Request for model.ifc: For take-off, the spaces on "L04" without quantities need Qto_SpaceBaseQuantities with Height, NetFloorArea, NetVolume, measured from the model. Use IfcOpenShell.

First a look at what the model holds.

```python
import ifcopenshell
import ifcopenshell.util.element
import ifcopenshell.util.unit

model = ifcopenshell.open("model.ifc")
print(model.schema)
for unit_type in ("LENGTHUNIT", "AREAUNIT", "VOLUMEUNIT"):
    print(unit_type, ifcopenshell.util.unit.calculate_unit_scale(model, unit_type))
storey = next(s for s in model.by_type("IfcBuildingStorey") if s.Name == "L04")
spaces = [e for e in ifcopenshell.util.element.get_decomposition(storey) if e.is_a("IfcSpace")]
for e in sorted(spaces, key=lambda e: e.id()):
    print(e.id(), e.is_a(), e.Name, list(ifcopenshell.util.element.get_psets(e, qtos_only=True)), sep=" | ")
```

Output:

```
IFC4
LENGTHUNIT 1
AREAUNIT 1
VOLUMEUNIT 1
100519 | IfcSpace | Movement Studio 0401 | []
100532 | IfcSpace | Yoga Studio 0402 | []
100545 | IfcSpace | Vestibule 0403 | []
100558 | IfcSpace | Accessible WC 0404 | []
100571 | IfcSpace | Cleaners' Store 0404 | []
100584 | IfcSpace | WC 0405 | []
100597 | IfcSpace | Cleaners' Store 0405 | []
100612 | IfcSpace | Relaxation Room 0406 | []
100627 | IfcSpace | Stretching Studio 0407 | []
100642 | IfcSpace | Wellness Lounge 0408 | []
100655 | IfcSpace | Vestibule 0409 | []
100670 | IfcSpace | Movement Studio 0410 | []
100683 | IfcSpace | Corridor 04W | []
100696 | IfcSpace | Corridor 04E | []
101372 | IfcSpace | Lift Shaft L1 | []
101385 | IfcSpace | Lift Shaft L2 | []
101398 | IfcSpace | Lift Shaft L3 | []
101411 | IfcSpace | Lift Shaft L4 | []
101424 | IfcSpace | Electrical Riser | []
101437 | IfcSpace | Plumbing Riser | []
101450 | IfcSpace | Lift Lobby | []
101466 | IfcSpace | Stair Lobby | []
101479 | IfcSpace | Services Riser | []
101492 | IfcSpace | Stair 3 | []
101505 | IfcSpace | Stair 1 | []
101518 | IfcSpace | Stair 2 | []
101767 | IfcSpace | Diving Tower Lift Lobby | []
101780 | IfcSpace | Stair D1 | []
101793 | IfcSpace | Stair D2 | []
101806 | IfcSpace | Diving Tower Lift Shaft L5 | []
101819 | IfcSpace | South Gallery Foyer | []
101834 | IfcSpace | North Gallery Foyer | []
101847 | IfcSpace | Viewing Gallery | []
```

```python
import ifcopenshell
import ifcopenshell.api.pset
import ifcopenshell.geom
import ifcopenshell.util.element
import ifcopenshell.util.shape
import ifcopenshell.util.unit

model = ifcopenshell.open("model.ifc")
unit_scale = ifcopenshell.util.unit.calculate_unit_scale(model)
area_scale = ifcopenshell.util.unit.calculate_unit_scale(model, "AREAUNIT")
volume_scale = ifcopenshell.util.unit.calculate_unit_scale(model, "VOLUMEUNIT")
settings = ifcopenshell.geom.settings()

storey = next(s for s in model.by_type("IfcBuildingStorey") if s.Name == "L04")
spaces = [e for e in ifcopenshell.util.element.get_decomposition(storey) if e.is_a("IfcSpace")]

for e in sorted(spaces, key=lambda e: e.id()):
    if ifcopenshell.util.element.get_psets(e, qtos_only=True, should_inherit=False):
        continue
    # Geometry comes back in metres, in the element's own axes.
    shape = ifcopenshell.geom.create_shape(settings, e)
    values = {
        "Height": ifcopenshell.util.shape.get_z(shape.geometry) / unit_scale,
        "NetFloorArea": ifcopenshell.util.shape.get_footprint_area(shape.geometry) / area_scale,
        "NetVolume": ifcopenshell.util.shape.get_volume(shape.geometry) / volume_scale,
    }
    qto = ifcopenshell.api.pset.add_qto(model, product=e, name="Qto_SpaceBaseQuantities")
    ifcopenshell.api.pset.edit_qto(model, qto=qto, properties=values)
    print(e.id(), {k: round(v, 3) for k, v in values.items()})

model.write("model-out.ifc")
```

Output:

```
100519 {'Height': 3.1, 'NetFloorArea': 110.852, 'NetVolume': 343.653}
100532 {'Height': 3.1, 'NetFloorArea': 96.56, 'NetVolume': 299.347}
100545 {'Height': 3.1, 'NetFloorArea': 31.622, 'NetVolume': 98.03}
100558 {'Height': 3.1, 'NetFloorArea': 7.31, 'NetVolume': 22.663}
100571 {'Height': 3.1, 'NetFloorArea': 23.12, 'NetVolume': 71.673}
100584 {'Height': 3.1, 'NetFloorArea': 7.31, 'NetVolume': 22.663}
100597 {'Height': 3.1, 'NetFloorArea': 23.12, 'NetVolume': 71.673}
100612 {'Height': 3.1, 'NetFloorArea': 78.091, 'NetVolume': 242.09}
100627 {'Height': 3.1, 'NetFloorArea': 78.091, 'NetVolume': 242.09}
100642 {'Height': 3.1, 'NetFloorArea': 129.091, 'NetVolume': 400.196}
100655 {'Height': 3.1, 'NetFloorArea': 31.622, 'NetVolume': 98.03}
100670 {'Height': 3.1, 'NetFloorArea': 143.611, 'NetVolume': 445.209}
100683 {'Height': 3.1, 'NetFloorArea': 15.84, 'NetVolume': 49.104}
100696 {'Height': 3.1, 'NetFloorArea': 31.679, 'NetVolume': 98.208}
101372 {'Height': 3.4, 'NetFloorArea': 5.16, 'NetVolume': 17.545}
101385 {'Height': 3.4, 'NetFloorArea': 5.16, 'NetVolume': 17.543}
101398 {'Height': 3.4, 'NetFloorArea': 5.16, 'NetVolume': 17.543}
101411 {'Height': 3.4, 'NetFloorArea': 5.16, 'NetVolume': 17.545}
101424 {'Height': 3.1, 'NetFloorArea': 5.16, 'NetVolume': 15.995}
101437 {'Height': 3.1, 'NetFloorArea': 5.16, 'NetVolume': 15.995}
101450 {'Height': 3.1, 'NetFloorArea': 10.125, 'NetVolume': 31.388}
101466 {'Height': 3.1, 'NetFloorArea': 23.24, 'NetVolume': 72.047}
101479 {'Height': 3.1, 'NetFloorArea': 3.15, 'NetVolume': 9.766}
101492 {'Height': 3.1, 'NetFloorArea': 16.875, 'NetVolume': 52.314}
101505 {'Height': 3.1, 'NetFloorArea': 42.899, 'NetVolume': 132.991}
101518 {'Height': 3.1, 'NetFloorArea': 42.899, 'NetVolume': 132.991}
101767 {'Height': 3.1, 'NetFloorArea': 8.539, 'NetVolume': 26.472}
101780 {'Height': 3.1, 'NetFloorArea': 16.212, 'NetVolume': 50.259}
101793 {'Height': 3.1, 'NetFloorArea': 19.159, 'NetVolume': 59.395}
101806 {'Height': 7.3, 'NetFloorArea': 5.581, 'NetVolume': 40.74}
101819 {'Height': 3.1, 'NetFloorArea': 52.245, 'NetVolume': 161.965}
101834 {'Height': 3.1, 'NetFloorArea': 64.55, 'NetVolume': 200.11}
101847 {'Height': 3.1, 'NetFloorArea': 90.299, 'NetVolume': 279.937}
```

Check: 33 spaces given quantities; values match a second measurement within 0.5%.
